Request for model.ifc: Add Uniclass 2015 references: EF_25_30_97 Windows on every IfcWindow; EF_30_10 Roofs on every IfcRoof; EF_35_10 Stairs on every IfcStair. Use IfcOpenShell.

First a look at what the model holds.

```python
import ifcopenshell

model = ifcopenshell.open("model.ifc")
print(model.schema)
print("classifications:", [c.Name for c in model.by_type("IfcClassification")])
for ifc_class in ("IfcDoor", "IfcRoof", "IfcStair", "IfcWall", "IfcWindow"):
    print(ifc_class, len(model.by_type(ifc_class)))
```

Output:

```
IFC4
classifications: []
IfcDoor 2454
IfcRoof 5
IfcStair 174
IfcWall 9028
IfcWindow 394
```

```python
import ifcopenshell
import ifcopenshell.api.classification

model = ifcopenshell.open("model.ifc")

system = ifcopenshell.api.classification.add_classification(model, classification="Uniclass 2015")

codes = {
    "IfcWindow": ("EF_25_30_97", "Windows"),
    "IfcRoof": ("EF_30_10", "Roofs"),
    "IfcStair": ("EF_35_10", "Stairs"),
}
for ifc_class, (code, name) in codes.items():
    products = model.by_type(ifc_class)
    ifcopenshell.api.classification.add_reference(
        model, products=products, classification=system, identification=code, name=name
    )
    print(code, len(products))

model.write("model-out.ifc")
```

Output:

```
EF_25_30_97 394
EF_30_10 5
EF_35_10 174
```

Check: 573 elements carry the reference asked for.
